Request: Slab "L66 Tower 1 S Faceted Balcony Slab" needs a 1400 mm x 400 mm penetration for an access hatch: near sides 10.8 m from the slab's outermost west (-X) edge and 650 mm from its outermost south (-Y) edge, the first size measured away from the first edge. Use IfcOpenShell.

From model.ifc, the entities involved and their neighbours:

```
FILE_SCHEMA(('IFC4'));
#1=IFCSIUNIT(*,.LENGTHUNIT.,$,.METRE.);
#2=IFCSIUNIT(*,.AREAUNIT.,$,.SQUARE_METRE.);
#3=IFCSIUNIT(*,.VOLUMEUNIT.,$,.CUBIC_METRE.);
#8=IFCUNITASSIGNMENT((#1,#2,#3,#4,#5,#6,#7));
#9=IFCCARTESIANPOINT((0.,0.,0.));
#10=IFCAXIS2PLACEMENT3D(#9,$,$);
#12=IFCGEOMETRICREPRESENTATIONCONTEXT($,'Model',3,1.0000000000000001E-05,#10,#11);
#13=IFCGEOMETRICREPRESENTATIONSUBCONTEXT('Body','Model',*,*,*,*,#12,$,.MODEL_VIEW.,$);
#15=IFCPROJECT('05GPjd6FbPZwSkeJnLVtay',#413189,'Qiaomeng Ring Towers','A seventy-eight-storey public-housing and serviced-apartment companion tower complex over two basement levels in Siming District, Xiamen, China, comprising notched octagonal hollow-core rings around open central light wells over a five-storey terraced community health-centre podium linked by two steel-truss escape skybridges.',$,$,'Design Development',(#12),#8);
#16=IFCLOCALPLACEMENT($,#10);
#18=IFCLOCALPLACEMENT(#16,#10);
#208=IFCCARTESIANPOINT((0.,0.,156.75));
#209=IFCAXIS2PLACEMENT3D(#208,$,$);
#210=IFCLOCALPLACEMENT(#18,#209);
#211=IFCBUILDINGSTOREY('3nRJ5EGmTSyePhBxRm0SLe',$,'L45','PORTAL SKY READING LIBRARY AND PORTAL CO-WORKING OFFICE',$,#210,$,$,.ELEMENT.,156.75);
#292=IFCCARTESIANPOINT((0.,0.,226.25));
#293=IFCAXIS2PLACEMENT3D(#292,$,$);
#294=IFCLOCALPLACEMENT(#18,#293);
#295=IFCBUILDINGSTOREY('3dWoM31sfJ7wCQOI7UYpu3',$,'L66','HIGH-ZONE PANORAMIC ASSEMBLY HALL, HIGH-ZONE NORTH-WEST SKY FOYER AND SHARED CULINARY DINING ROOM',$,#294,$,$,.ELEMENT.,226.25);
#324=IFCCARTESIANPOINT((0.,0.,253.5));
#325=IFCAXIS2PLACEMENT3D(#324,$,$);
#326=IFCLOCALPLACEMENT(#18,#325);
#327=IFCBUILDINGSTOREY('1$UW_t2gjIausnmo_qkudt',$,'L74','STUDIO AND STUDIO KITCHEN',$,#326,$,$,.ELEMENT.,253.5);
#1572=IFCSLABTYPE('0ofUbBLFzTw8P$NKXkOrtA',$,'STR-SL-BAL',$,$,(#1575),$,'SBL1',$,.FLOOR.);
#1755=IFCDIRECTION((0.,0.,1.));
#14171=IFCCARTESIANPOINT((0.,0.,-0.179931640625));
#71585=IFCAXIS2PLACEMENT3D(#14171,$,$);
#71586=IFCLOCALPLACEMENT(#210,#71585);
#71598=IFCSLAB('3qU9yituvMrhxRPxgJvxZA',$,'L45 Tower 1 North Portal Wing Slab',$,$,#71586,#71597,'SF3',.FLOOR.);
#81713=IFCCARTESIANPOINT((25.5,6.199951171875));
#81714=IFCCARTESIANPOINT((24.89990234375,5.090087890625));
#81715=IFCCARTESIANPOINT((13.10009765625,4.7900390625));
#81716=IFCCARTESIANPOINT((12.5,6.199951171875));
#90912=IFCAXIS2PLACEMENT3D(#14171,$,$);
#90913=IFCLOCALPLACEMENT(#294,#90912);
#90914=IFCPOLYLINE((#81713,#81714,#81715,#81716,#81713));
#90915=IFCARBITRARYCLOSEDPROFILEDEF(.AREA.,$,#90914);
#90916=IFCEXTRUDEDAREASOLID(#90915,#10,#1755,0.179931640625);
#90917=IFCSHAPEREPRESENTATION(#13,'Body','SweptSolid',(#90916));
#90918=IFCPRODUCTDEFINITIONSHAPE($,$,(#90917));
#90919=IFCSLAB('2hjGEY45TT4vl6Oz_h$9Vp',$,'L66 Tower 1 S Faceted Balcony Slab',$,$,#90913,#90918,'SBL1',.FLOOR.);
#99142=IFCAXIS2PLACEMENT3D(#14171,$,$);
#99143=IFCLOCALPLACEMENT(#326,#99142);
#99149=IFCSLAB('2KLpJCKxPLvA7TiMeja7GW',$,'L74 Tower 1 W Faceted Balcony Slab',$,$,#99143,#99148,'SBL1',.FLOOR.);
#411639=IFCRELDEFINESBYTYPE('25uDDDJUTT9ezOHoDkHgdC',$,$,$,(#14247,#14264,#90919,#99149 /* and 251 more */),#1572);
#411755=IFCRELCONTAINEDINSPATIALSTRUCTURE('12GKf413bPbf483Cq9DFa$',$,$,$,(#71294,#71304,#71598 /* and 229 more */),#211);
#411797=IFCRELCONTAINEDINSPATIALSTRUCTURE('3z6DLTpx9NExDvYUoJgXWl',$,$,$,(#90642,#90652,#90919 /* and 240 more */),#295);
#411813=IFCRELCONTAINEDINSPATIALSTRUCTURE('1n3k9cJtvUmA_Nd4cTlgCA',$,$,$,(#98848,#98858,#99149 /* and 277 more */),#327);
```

```python
import numpy as np
import ifcopenshell
import ifcopenshell.api.feature
import ifcopenshell.api.geometry
import ifcopenshell.api.root
import ifcopenshell.geom
import ifcopenshell.util.placement
import ifcopenshell.util.representation
import ifcopenshell.util.shape
import ifcopenshell.util.unit

model = ifcopenshell.open("model.ifc")
unit_scale = ifcopenshell.util.unit.calculate_unit_scale(model)
settings = ifcopenshell.geom.settings()


def volume(element):
    """Net volume in cubic metres, openings subtracted."""
    shape = ifcopenshell.geom.create_shape(settings, element)
    return ifcopenshell.util.shape.get_volume(shape.geometry)


slab = model.by_guid("2hjGEY45TT4vl6Oz_h$9Vp")
before = volume(slab)

# Extent in the slab's own axes, in metres. The edges named are its -X and -Y sides.
slab_shape = ifcopenshell.geom.create_shape(settings, slab)
vertices = ifcopenshell.util.shape.get_vertices(slab_shape.geometry)
x_min, y_min, bottom = vertices.min(axis=0)
top = vertices[:, 2].max()

opening = ifcopenshell.api.root.create_entity(model, ifc_class="IfcOpeningElement", name="Access hatch opening", predefined_type="OPENING")
context = ifcopenshell.util.representation.get_context(model, "Model", "Body", "MODEL_VIEW")
width, depth = 1.4, 0.4
outline = [(0.0, 0.0), (width, 0.0), (width, depth), (0.0, depth), (0.0, 0.0)]
# Overshoot both faces by 50 mm so the cut is clean.
shape = ifcopenshell.api.geometry.add_slab_representation(
    model, context=context, depth=top - bottom + 0.1, polyline=outline
)
ifcopenshell.api.geometry.assign_representation(model, product=opening, representation=shape)

matrix = ifcopenshell.util.placement.get_local_placement(slab.ObjectPlacement)
matrix[:, 3] = matrix @ np.append(np.array([x_min + 10.8, y_min + 0.65, bottom - 0.05]) / unit_scale, 1.0)
ifcopenshell.api.geometry.edit_object_placement(model, product=opening, matrix=matrix, is_si=False)
ifcopenshell.api.feature.add_feature(model, feature=opening, element=slab)

after = volume(slab)

print(f"slab volume {before:.3f} -> {after:.3f} m3")

model.write("model_updated.ifc")
```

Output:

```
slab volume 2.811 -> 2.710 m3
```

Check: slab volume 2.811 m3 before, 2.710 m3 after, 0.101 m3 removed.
